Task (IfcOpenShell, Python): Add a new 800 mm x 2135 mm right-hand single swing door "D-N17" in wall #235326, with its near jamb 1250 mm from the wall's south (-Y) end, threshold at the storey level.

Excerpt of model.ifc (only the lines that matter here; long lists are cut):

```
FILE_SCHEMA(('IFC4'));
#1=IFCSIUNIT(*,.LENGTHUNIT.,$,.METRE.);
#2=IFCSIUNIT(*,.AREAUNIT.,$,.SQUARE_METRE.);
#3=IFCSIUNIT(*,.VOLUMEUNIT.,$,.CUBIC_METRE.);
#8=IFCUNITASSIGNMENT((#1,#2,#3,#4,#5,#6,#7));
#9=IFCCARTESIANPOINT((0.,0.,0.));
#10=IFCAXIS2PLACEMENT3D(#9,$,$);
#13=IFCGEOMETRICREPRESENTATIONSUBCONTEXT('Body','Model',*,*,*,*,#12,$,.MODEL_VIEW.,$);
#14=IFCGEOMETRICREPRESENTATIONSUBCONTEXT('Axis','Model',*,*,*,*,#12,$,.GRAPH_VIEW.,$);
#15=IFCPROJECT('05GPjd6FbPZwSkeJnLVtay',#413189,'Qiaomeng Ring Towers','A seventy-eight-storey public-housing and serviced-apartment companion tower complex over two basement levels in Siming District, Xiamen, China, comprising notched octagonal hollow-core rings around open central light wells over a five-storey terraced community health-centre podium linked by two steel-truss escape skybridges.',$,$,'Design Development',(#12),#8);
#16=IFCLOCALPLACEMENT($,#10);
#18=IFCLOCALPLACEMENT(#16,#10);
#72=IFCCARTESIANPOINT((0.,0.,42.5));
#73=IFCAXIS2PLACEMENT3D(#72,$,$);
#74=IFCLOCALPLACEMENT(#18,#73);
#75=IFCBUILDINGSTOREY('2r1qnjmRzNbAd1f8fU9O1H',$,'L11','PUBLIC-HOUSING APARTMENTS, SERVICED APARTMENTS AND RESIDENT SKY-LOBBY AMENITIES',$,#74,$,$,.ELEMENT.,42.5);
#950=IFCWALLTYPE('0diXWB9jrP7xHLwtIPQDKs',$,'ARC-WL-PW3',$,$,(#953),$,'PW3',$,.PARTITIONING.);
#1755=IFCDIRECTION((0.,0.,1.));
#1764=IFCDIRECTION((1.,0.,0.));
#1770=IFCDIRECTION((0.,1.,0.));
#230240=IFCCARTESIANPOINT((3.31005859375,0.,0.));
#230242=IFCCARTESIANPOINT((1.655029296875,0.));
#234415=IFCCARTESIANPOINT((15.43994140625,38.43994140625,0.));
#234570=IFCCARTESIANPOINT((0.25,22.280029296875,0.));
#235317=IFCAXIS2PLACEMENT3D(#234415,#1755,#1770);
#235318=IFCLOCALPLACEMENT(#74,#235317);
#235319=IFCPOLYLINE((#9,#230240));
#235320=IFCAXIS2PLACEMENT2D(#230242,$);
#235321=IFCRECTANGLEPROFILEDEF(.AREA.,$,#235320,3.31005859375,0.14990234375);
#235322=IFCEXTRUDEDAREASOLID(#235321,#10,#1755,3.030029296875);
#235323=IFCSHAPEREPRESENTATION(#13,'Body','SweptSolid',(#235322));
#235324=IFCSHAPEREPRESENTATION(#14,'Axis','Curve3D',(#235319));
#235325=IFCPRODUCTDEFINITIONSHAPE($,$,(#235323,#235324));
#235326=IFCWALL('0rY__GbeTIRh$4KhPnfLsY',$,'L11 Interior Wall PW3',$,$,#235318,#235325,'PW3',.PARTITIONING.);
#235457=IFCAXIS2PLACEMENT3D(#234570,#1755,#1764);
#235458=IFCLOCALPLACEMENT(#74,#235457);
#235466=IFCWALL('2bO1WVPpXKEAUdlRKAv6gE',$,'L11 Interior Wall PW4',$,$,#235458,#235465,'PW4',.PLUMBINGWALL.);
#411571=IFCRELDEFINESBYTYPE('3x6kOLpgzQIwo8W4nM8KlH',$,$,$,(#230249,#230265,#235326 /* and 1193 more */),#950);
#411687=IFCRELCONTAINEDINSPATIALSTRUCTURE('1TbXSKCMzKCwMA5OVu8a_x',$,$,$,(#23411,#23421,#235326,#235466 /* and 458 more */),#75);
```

```python
import numpy as np
import ifcopenshell
import ifcopenshell.api.feature
import ifcopenshell.api.geometry
import ifcopenshell.api.root
import ifcopenshell.api.spatial
import ifcopenshell.geom
import ifcopenshell.util.element
import ifcopenshell.util.placement
import ifcopenshell.util.representation
import ifcopenshell.util.shape
import ifcopenshell.util.unit

model = ifcopenshell.open("model.ifc")
unit_scale = ifcopenshell.util.unit.calculate_unit_scale(model)
settings = ifcopenshell.geom.settings()


def volume(element):
    """Net volume in cubic metres, openings subtracted."""
    shape = ifcopenshell.geom.create_shape(settings, element)
    return ifcopenshell.util.shape.get_volume(shape.geometry)


wall = model.by_guid("0rY__GbeTIRh$4KhPnfLsY")
storey = ifcopenshell.util.element.get_container(wall, ifc_class="IfcBuildingStorey")
context = ifcopenshell.util.representation.get_context(model, "Model", "Body", "MODEL_VIEW")
before = volume(wall)

width, height, from_end, sill = 0.8, 2.135, 1.25, 0.0  # metres

# The wall runs along its own X axis, and the end named is its -X end.
wall_shape = ifcopenshell.geom.create_shape(settings, wall)
x, y, z = ifcopenshell.util.shape.get_vertices(wall_shape.geometry).T
start = x.min() + from_end
face, thickness = float(y.min()), float(y.max() - y.min())
wall_matrix = ifcopenshell.util.placement.get_local_placement(wall.ObjectPlacement)
level = ifcopenshell.util.placement.get_local_placement(storey.ObjectPlacement)[2, 3]


def in_wall(x, y):
    """Placement at x, y metres in the wall's axes, at sill height."""
    matrix = wall_matrix.copy()
    matrix[:, 3] = wall_matrix @ np.array([x / unit_scale, y / unit_scale, 0.0, 1.0])
    matrix[2, 3] = level + sill / unit_scale
    return matrix


# Opening: a box that overshoots both wall faces by 50 mm.
opening = ifcopenshell.api.root.create_entity(model, ifc_class="IfcOpeningElement", predefined_type="OPENING")
box = ifcopenshell.api.geometry.add_wall_representation(
    model, context=context, length=width, height=height, thickness=thickness + 0.1
)
ifcopenshell.api.geometry.assign_representation(model, product=opening, representation=box)
ifcopenshell.api.geometry.edit_object_placement(model, product=opening, matrix=in_wall(start, face - 0.05), is_si=False)
ifcopenshell.api.feature.add_feature(model, feature=opening, element=wall)

door = ifcopenshell.api.root.create_entity(model, ifc_class="IfcDoor", name="D-N17", predefined_type="DOOR")
door.OverallWidth, door.OverallHeight = width / unit_scale, height / unit_scale
door.OperationType = "SINGLE_SWING_RIGHT"
body = ifcopenshell.api.geometry.add_door_representation(
    model,
    context=context,
    overall_width=door.OverallWidth,
    overall_height=door.OverallHeight,
    operation_type="SINGLE_SWING_RIGHT",
    lining_properties={"LiningDepth": thickness / unit_scale, "ThresholdDepth": thickness / unit_scale},
)
ifcopenshell.api.geometry.assign_representation(model, product=door, representation=body)
ifcopenshell.api.spatial.assign_container(model, products=[door], relating_structure=storey)
ifcopenshell.api.feature.add_filling(model, opening=opening, element=door)

# The lining spans the wall, so the door starts at the wall face.
ifcopenshell.api.geometry.edit_object_placement(model, product=door, matrix=in_wall(start, face), is_si=False)

after = volume(wall)

print(f"wall volume {before:.3f} -> {after:.3f} m3")

model.write("model_updated.ifc")
```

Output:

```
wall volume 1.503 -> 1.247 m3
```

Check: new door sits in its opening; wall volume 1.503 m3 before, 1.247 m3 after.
